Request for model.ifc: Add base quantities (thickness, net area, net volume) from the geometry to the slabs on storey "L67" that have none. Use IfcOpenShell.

First a look at what the model holds.

```python
import ifcopenshell
import ifcopenshell.util.element
import ifcopenshell.util.unit

model = ifcopenshell.open("model.ifc")
print(model.schema)
for unit_type in ("LENGTHUNIT", "AREAUNIT", "VOLUMEUNIT"):
    print(unit_type, ifcopenshell.util.unit.calculate_unit_scale(model, unit_type))
storey = next(s for s in model.by_type("IfcBuildingStorey") if s.Name == "L67")
slabs = [e for e in ifcopenshell.util.element.get_decomposition(storey) if e.is_a("IfcSlab")]
for e in sorted(slabs, key=lambda e: e.id()):
    print(e.id(), e.is_a(), e.Name, list(ifcopenshell.util.element.get_psets(e, qtos_only=True)), sep=" | ")
```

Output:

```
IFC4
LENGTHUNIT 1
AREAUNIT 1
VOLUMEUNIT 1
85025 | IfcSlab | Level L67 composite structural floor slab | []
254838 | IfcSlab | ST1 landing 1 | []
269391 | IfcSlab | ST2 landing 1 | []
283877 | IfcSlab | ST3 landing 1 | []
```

```python
import ifcopenshell
import ifcopenshell.api.pset
import ifcopenshell.geom
import ifcopenshell.util.element
import ifcopenshell.util.shape
import ifcopenshell.util.unit

model = ifcopenshell.open("model.ifc")
unit_scale = ifcopenshell.util.unit.calculate_unit_scale(model)
area_scale = ifcopenshell.util.unit.calculate_unit_scale(model, "AREAUNIT")
volume_scale = ifcopenshell.util.unit.calculate_unit_scale(model, "VOLUMEUNIT")
settings = ifcopenshell.geom.settings()

storey = next(s for s in model.by_type("IfcBuildingStorey") if s.Name == "L67")
slabs = [e for e in ifcopenshell.util.element.get_decomposition(storey) if e.is_a("IfcSlab")]

for e in sorted(slabs, key=lambda e: e.id()):
    if ifcopenshell.util.element.get_psets(e, qtos_only=True, should_inherit=False):
        continue
    # Geometry comes back in metres, in the element's own axes.
    shape = ifcopenshell.geom.create_shape(settings, e)
    values = {
        "Width": ifcopenshell.util.shape.get_z(shape.geometry) / unit_scale,
        "NetArea": ifcopenshell.util.shape.get_footprint_area(shape.geometry) / area_scale,
        "NetVolume": ifcopenshell.util.shape.get_volume(shape.geometry) / volume_scale,
    }
    qto = ifcopenshell.api.pset.add_qto(model, product=e, name="Qto_SlabBaseQuantities")
    ifcopenshell.api.pset.edit_qto(model, qto=qto, properties=values)
    print(e.id(), {k: round(v, 3) for k, v in values.items()})

model.write("model_updated.ifc")
```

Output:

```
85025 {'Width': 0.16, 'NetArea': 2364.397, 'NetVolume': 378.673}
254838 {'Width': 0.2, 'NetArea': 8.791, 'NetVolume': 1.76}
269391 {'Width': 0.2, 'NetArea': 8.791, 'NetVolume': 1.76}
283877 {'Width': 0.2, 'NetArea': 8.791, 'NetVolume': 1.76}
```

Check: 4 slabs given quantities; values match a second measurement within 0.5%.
